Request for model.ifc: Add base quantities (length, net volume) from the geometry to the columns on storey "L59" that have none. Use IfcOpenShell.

First a look at what the model holds.

```python
import ifcopenshell
import ifcopenshell.util.element
import ifcopenshell.util.unit

model = ifcopenshell.open("model.ifc")
print(model.schema)
for unit_type in ("LENGTHUNIT", "AREAUNIT", "VOLUMEUNIT"):
    print(unit_type, ifcopenshell.util.unit.calculate_unit_scale(model, unit_type))
storey = next(s for s in model.by_type("IfcBuildingStorey") if s.Name == "L59")
columns = [e for e in ifcopenshell.util.element.get_decomposition(storey) if e.is_a("IfcColumn")]
for e in sorted(columns, key=lambda e: e.id()):
    print(e.id(), e.is_a(), e.Name, list(ifcopenshell.util.element.get_psets(e, qtos_only=True)), sep=" | ")
```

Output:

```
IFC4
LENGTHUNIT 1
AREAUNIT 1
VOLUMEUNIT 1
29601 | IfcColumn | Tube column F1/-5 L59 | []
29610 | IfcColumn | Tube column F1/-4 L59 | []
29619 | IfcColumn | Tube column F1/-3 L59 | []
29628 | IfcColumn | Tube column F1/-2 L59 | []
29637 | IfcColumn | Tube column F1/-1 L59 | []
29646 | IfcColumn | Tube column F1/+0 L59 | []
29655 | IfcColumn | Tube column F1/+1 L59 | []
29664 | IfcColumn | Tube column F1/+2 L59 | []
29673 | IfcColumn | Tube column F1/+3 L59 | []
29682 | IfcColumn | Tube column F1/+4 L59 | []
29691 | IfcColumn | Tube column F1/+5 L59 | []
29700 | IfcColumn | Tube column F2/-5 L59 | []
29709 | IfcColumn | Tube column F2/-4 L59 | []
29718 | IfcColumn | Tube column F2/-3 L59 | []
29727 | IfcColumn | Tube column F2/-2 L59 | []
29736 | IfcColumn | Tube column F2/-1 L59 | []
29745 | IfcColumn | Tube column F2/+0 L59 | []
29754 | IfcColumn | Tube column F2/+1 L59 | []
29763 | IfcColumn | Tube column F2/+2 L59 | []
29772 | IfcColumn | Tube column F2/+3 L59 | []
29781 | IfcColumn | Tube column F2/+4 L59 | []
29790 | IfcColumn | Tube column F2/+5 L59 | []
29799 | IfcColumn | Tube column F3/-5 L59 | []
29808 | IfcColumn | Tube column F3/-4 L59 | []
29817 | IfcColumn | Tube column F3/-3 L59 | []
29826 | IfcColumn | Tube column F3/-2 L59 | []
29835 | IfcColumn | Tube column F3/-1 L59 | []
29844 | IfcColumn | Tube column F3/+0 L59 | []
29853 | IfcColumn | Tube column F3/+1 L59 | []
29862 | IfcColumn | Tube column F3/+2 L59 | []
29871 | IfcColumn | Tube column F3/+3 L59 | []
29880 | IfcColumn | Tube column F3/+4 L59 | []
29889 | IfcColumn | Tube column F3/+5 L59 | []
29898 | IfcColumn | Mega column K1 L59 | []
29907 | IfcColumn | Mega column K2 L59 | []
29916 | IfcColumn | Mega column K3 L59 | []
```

```python
import ifcopenshell
import ifcopenshell.api.pset
import ifcopenshell.geom
import ifcopenshell.util.element
import ifcopenshell.util.shape
import ifcopenshell.util.unit

model = ifcopenshell.open("model.ifc")
unit_scale = ifcopenshell.util.unit.calculate_unit_scale(model)
volume_scale = ifcopenshell.util.unit.calculate_unit_scale(model, "VOLUMEUNIT")
settings = ifcopenshell.geom.settings()

storey = next(s for s in model.by_type("IfcBuildingStorey") if s.Name == "L59")
columns = [e for e in ifcopenshell.util.element.get_decomposition(storey) if e.is_a("IfcColumn")]

for e in sorted(columns, key=lambda e: e.id()):
    if ifcopenshell.util.element.get_psets(e, qtos_only=True, should_inherit=False):
        continue
    # Geometry comes back in metres, in the element's own axes.
    shape = ifcopenshell.geom.create_shape(settings, e)
    values = {
        "Length": ifcopenshell.util.shape.get_z(shape.geometry) / unit_scale,
        "NetVolume": ifcopenshell.util.shape.get_volume(shape.geometry) / volume_scale,
    }
    qto = ifcopenshell.api.pset.add_qto(model, product=e, name="Qto_ColumnBaseQuantities")
    ifcopenshell.api.pset.edit_qto(model, qto=qto, properties=values)
    print(e.id(), {k: round(v, 3) for k, v in values.items()})

model.write("model_edited.ifc")
```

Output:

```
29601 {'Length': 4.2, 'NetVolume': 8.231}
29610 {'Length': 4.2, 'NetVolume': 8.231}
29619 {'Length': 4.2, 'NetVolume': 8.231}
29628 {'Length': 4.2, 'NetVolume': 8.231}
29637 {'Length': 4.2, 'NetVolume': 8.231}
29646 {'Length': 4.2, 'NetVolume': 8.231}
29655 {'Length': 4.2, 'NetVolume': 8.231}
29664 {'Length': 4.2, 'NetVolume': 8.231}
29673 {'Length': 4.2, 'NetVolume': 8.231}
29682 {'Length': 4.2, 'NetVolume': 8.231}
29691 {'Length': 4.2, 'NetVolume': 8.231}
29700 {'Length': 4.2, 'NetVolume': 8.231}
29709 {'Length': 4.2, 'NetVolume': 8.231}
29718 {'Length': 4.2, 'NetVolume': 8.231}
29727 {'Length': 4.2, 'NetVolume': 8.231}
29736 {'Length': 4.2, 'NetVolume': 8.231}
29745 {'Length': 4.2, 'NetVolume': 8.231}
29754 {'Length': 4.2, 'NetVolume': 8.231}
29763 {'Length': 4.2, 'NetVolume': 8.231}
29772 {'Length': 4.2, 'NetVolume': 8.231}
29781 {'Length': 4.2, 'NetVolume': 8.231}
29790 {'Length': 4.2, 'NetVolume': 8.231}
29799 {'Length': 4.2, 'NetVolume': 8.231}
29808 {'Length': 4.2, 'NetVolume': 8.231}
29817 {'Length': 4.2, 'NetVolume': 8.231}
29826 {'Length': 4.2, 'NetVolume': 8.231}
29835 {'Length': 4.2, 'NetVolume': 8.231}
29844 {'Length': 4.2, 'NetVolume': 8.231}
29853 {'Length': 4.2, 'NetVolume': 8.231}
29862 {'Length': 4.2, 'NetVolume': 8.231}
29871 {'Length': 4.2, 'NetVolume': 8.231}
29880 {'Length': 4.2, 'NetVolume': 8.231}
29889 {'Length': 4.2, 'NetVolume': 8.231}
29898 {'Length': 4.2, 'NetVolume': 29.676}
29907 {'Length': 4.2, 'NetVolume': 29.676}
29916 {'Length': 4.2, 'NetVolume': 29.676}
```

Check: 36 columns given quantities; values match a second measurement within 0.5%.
